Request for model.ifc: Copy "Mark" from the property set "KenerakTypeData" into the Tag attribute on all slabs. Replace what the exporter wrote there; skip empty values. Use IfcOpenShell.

First a look at what the model holds.

```python
import ifcopenshell
import ifcopenshell.util.element

model = ifcopenshell.open("model.ifc")
print(model.schema)
slabs = model.by_type("IfcSlab")
print(len(slabs), "slabs")
for e in slabs[:8]:
    source = ifcopenshell.util.element.get_pset(e, "KenerakTypeData", "Mark")
    target = e.Tag
    print(e.id(), repr(source), repr(target), sep=" | ")
```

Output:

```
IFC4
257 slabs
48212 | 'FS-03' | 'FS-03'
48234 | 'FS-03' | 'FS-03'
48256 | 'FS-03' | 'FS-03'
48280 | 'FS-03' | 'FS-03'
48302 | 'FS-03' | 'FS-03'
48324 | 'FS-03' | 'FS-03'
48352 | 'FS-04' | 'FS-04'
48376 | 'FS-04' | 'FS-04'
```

```python
import ifcopenshell
import ifcopenshell.util.element

model = ifcopenshell.open("model.ifc")

count = 0
for e in model.by_type("IfcSlab"):
    value = ifcopenshell.util.element.get_pset(e, "KenerakTypeData", "Mark")
    current = e.Tag
    if not value or not value.strip() or current == value:
        continue
    e.Tag = value
    count += 1

print(count, "slabs updated")

model.write("model_v2.ifc")
```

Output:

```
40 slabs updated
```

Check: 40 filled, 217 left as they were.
